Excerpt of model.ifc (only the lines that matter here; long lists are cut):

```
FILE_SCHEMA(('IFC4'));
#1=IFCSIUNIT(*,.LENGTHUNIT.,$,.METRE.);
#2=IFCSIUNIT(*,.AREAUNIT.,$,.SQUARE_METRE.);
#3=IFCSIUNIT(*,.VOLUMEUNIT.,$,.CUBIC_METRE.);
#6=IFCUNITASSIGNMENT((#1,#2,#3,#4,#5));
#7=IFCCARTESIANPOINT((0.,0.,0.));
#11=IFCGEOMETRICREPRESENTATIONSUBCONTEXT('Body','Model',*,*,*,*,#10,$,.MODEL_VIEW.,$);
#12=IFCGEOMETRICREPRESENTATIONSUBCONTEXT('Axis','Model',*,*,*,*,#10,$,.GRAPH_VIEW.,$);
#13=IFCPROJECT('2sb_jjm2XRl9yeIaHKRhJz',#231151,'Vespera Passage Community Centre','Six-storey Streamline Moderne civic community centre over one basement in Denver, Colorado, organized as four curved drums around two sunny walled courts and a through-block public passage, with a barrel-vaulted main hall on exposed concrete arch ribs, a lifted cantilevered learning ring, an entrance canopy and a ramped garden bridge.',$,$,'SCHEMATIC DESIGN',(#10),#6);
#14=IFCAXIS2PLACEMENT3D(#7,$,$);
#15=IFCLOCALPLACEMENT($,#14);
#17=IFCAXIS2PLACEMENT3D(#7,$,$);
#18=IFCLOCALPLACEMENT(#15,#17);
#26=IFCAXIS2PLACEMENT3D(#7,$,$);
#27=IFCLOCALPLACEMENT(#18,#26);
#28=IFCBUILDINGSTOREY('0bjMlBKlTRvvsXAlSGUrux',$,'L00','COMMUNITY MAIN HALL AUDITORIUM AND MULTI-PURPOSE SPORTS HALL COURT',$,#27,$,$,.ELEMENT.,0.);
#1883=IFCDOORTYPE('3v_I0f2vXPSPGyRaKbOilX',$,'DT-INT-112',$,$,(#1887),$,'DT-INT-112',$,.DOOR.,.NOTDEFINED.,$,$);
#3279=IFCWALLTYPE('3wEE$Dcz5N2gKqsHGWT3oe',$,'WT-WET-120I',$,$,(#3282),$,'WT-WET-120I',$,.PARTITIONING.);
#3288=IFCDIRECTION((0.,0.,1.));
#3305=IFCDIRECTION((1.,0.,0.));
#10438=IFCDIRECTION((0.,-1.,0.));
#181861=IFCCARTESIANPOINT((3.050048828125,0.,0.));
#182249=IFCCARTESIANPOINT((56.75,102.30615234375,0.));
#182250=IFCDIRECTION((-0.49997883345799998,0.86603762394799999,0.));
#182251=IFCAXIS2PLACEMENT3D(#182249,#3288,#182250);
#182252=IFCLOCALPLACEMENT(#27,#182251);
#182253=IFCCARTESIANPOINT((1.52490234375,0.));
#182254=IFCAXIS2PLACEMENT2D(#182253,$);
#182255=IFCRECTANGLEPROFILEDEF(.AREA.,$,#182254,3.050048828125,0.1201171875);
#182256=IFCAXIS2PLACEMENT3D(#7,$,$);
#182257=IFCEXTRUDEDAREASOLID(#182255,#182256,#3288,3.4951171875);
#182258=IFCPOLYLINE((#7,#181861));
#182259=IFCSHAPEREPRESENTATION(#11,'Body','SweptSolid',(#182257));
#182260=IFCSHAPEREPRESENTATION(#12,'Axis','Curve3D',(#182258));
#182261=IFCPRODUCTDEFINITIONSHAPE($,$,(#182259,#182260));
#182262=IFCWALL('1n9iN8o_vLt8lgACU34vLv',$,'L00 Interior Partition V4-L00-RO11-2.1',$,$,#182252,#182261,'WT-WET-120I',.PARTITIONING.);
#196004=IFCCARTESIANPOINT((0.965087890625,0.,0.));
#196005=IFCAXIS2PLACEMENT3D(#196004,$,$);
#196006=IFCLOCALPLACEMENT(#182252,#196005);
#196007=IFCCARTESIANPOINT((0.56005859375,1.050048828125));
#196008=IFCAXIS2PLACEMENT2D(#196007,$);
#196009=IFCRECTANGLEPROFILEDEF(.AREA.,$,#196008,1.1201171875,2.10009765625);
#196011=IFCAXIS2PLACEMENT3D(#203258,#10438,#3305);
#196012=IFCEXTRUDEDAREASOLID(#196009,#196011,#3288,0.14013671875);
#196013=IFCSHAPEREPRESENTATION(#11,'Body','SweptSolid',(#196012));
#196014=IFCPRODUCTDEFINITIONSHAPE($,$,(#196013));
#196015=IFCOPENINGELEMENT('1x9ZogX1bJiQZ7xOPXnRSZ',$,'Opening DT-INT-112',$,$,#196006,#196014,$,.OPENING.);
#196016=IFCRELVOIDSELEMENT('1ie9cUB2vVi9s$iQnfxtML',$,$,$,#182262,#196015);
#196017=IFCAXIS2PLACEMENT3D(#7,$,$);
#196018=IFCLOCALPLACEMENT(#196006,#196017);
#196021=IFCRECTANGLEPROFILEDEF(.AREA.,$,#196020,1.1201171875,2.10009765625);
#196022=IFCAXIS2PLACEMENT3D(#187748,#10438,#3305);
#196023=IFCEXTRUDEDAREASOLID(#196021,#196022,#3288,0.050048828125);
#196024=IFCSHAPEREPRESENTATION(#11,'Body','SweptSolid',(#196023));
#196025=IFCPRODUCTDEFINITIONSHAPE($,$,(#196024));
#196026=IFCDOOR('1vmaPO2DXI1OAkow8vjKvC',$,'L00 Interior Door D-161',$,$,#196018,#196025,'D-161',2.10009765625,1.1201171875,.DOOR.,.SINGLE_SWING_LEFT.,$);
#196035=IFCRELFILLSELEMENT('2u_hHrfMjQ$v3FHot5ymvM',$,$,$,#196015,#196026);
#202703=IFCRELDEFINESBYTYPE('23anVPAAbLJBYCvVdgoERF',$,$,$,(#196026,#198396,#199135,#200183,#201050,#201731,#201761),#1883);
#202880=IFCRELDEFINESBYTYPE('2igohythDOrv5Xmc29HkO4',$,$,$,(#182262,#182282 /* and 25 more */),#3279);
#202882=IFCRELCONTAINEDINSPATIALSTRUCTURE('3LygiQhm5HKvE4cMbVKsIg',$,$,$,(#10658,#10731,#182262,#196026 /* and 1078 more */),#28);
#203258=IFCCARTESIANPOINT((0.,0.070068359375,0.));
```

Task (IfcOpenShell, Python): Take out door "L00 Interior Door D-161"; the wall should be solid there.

```python
import ifcopenshell
import ifcopenshell.api.feature
import ifcopenshell.api.root
import ifcopenshell.geom
import ifcopenshell.util.shape

model = ifcopenshell.open("model.ifc")
settings = ifcopenshell.geom.settings()


def volume(element):
    """Net volume in cubic metres, openings subtracted."""
    shape = ifcopenshell.geom.create_shape(settings, element)
    return ifcopenshell.util.shape.get_volume(shape.geometry)


door = model.by_id(196026)
opening = door.FillsVoids[0].RelatingOpeningElement
wall = opening.VoidsElements[0].RelatingBuildingElement
before = volume(wall)

ifcopenshell.api.root.remove_product(model, product=door)
ifcopenshell.api.feature.remove_feature(model, feature=opening)

after = volume(wall)

print(f"wall volume {before:.3f} -> {after:.3f} m3")

model.write("model-out.ifc")
```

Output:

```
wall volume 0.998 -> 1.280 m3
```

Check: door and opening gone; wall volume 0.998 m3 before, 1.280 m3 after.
